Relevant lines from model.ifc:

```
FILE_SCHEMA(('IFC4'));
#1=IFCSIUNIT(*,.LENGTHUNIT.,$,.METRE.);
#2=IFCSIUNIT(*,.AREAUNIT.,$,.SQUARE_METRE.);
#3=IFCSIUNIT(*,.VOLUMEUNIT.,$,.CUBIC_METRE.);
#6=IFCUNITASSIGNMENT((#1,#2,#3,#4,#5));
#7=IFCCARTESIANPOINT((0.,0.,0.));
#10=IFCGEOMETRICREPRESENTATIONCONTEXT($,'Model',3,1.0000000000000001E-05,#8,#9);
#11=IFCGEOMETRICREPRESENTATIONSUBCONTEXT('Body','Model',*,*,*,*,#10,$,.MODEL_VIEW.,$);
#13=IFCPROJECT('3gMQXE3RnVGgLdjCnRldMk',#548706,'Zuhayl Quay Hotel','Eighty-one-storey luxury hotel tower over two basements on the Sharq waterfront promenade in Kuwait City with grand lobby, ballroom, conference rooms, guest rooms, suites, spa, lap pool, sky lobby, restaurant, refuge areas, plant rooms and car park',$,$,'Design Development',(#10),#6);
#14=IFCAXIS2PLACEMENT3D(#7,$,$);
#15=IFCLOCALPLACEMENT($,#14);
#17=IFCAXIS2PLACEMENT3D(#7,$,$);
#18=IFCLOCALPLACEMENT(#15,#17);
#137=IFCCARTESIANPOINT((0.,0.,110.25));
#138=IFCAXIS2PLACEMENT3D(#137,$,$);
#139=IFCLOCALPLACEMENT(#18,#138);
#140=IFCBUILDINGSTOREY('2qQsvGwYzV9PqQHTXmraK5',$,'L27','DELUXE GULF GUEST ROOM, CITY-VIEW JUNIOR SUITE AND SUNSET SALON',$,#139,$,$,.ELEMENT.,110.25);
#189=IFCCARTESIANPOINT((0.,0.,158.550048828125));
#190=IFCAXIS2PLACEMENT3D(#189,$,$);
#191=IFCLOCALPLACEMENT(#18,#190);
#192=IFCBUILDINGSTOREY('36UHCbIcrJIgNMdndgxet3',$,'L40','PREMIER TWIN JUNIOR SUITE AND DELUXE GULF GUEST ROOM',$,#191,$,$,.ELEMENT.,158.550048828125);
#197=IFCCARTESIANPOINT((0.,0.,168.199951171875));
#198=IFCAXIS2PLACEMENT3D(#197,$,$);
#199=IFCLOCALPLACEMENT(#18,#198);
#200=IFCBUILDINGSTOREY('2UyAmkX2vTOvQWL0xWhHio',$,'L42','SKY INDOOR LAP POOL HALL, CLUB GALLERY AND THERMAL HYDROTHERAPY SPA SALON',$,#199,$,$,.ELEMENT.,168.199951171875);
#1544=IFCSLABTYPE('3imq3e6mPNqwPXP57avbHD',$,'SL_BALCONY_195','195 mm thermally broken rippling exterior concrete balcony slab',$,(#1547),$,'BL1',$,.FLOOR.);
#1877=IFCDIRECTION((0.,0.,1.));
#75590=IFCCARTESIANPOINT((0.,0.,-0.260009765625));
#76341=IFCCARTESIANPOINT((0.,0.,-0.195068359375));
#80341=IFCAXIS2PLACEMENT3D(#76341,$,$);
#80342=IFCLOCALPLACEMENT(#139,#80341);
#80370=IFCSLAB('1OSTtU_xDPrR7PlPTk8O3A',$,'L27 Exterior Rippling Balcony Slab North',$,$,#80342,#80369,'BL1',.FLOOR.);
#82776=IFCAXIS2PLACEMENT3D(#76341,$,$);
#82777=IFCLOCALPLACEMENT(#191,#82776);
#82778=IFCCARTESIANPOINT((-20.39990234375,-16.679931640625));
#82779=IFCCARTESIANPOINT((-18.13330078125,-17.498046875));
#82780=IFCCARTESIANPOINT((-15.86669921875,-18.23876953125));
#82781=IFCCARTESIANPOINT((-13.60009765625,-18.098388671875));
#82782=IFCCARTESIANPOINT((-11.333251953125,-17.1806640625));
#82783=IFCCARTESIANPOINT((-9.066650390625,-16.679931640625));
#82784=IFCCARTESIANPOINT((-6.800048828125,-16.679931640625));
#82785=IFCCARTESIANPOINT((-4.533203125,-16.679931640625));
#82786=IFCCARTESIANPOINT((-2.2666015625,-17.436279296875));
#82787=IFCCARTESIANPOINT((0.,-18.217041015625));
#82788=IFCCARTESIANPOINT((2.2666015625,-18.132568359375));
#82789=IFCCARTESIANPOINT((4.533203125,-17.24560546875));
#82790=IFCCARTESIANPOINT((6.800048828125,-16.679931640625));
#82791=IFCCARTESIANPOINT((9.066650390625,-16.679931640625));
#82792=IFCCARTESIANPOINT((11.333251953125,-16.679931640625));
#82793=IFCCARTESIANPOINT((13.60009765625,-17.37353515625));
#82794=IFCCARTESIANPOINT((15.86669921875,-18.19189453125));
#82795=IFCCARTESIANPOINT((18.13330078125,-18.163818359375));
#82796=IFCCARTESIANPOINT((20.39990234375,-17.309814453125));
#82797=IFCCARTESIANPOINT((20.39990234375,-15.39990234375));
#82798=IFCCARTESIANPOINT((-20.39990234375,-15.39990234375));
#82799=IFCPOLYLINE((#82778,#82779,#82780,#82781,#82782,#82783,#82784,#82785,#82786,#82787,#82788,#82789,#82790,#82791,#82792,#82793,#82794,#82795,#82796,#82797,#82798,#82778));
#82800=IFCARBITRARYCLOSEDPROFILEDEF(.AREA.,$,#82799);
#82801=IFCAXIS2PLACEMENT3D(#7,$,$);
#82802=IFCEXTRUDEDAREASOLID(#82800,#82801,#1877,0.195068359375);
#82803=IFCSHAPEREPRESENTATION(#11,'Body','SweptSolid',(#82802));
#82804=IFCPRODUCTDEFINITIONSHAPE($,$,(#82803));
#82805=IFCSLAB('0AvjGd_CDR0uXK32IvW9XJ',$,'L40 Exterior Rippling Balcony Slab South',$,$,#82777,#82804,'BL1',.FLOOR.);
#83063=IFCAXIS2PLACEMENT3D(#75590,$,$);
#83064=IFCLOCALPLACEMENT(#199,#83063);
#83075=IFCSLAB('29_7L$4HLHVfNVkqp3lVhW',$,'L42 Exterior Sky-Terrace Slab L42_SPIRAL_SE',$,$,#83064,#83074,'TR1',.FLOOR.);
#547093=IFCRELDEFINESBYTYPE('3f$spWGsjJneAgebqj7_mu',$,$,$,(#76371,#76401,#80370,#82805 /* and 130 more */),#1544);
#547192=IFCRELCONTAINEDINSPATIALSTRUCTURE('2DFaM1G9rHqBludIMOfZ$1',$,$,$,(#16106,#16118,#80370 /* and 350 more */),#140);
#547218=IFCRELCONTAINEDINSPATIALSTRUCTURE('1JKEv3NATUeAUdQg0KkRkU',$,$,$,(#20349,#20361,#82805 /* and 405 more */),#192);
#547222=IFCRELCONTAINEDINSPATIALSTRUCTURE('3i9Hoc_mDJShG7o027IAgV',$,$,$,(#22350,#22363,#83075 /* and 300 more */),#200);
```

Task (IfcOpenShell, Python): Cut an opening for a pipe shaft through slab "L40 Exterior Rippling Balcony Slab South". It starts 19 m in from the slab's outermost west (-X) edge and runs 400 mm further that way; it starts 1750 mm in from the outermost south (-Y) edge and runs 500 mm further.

```python
import numpy as np
import ifcopenshell
import ifcopenshell.api.feature
import ifcopenshell.api.geometry
import ifcopenshell.api.root
import ifcopenshell.geom
import ifcopenshell.util.placement
import ifcopenshell.util.representation
import ifcopenshell.util.shape
import ifcopenshell.util.unit

model = ifcopenshell.open("model.ifc")
unit_scale = ifcopenshell.util.unit.calculate_unit_scale(model)
settings = ifcopenshell.geom.settings()


def volume(element):
    """Net volume in cubic metres, openings subtracted."""
    shape = ifcopenshell.geom.create_shape(settings, element)
    return ifcopenshell.util.shape.get_volume(shape.geometry)


slab = model.by_guid("0AvjGd_CDR0uXK32IvW9XJ")
before = volume(slab)

# Extent in the slab's own axes, in metres. The edges named are its -X and -Y sides.
slab_shape = ifcopenshell.geom.create_shape(settings, slab)
vertices = ifcopenshell.util.shape.get_vertices(slab_shape.geometry)
x_min, y_min, bottom = vertices.min(axis=0)
top = vertices[:, 2].max()

opening = ifcopenshell.api.root.create_entity(model, ifc_class="IfcOpeningElement", name="Pipe shaft opening", predefined_type="OPENING")
context = ifcopenshell.util.representation.get_context(model, "Model", "Body", "MODEL_VIEW")
width, depth = 0.4, 0.5
outline = [(0.0, 0.0), (width, 0.0), (width, depth), (0.0, depth), (0.0, 0.0)]
# Overshoot both faces by 50 mm so the cut is clean.
shape = ifcopenshell.api.geometry.add_slab_representation(
    model, context=context, depth=top - bottom + 0.1, polyline=outline
)
ifcopenshell.api.geometry.assign_representation(model, product=opening, representation=shape)

matrix = ifcopenshell.util.placement.get_local_placement(slab.ObjectPlacement)
matrix[:, 3] = matrix @ np.append(np.array([x_min + 19, y_min + 1.75, bottom - 0.05]) / unit_scale, 1.0)
ifcopenshell.api.geometry.edit_object_placement(model, product=opening, matrix=matrix, is_si=False)
ifcopenshell.api.feature.add_feature(model, feature=opening, element=slab)

after = volume(slab)

print(f"slab volume {before:.3f} -> {after:.3f} m3")

model.write("model_rev.ifc")
```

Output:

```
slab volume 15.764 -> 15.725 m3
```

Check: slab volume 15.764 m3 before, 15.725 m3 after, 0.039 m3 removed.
